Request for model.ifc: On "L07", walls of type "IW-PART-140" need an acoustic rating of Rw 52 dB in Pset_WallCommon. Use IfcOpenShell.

First a look at what the model holds.

```python
import ifcopenshell
import ifcopenshell.util.element

model = ifcopenshell.open("model.ifc")
print(model.schema)
storey = next(s for s in model.by_type("IfcBuildingStorey") if s.Name == "L07")
walls = [e for e in ifcopenshell.util.element.get_decomposition(storey) if e.is_a("IfcWall")]
seen = {}
for e in walls:
    element_type = ifcopenshell.util.element.get_type(e)
    key = (element_type.Name if element_type != e and element_type else None, ifcopenshell.util.element.get_pset(e, "Pset_WallCommon", "AcousticRating"))
    seen[key] = seen.get(key, 0) + 1
for (name, value), count in sorted(seen.items(), key=str):
    print(count, "x", name, "|", value)
```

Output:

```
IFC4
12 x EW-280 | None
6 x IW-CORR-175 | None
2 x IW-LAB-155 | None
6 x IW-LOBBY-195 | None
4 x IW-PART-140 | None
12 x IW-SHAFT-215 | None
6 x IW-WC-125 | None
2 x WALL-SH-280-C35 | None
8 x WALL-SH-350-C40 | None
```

```python
import ifcopenshell
import ifcopenshell.api.pset
import ifcopenshell.util.element

model = ifcopenshell.open("model.ifc")

storey = next(s for s in model.by_type("IfcBuildingStorey") if s.Name == "L07")
walls = [e for e in ifcopenshell.util.element.get_decomposition(storey) if e.is_a("IfcWall")]

count = 0
for e in walls:
    element_type = ifcopenshell.util.element.get_type(e)
    if element_type in (None, e) or element_type.Name != "IW-PART-140":
        continue
    # add_pset returns the element's existing set when there is one.
    pset = ifcopenshell.api.pset.add_pset(model, product=e, name="Pset_WallCommon")
    ifcopenshell.api.pset.edit_pset(model, pset=pset, properties={"AcousticRating": "Rw 52 dB"})
    count += 1

print(count, "walls updated")

model.write("model_rev.ifc")
```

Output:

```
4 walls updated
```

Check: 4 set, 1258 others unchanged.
